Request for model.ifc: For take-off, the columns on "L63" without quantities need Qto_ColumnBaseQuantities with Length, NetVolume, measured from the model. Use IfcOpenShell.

First a look at what the model holds.

```python
import ifcopenshell
import ifcopenshell.util.element
import ifcopenshell.util.unit

model = ifcopenshell.open("model.ifc")
print(model.schema)
for unit_type in ("LENGTHUNIT", "AREAUNIT", "VOLUMEUNIT"):
    print(unit_type, ifcopenshell.util.unit.calculate_unit_scale(model, unit_type))
storey = next(s for s in model.by_type("IfcBuildingStorey") if s.Name == "L63")
columns = [e for e in ifcopenshell.util.element.get_decomposition(storey) if e.is_a("IfcColumn")]
for e in sorted(columns, key=lambda e: e.id()):
    print(e.id(), e.is_a(), e.Name, list(ifcopenshell.util.element.get_psets(e, qtos_only=True)), sep=" | ")
```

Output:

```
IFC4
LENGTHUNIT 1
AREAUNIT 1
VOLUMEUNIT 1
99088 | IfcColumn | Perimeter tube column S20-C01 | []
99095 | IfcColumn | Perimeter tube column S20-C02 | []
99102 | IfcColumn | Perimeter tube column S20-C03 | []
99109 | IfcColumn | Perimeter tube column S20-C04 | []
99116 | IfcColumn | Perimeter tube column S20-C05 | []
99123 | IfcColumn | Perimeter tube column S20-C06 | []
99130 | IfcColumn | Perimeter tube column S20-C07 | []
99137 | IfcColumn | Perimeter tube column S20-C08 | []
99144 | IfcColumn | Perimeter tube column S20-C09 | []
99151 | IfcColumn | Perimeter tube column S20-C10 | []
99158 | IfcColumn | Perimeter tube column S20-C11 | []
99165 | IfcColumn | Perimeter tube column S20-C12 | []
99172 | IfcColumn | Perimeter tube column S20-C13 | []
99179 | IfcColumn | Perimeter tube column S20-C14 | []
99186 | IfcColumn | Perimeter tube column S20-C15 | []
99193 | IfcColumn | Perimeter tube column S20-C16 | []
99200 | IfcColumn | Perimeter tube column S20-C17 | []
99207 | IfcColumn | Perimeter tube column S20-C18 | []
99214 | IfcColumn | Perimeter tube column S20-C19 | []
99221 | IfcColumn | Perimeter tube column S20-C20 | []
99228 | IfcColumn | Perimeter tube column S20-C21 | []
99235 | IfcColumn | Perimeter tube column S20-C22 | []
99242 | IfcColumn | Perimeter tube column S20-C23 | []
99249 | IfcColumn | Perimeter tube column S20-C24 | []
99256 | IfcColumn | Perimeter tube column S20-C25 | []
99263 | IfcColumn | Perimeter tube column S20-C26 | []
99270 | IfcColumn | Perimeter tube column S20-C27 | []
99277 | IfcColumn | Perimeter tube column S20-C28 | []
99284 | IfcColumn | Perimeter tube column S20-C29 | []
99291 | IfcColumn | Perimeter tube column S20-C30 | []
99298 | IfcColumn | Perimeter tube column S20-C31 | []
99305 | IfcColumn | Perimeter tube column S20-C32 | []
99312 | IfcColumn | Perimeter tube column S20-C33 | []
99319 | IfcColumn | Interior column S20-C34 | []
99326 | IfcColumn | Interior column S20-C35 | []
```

```python
import ifcopenshell
import ifcopenshell.api.pset
import ifcopenshell.geom
import ifcopenshell.util.element
import ifcopenshell.util.shape
import ifcopenshell.util.unit

model = ifcopenshell.open("model.ifc")
unit_scale = ifcopenshell.util.unit.calculate_unit_scale(model)
volume_scale = ifcopenshell.util.unit.calculate_unit_scale(model, "VOLUMEUNIT")
settings = ifcopenshell.geom.settings()

storey = next(s for s in model.by_type("IfcBuildingStorey") if s.Name == "L63")
columns = [e for e in ifcopenshell.util.element.get_decomposition(storey) if e.is_a("IfcColumn")]

for e in sorted(columns, key=lambda e: e.id()):
    if ifcopenshell.util.element.get_psets(e, qtos_only=True, should_inherit=False):
        continue
    # Geometry comes back in metres, in the element's own axes.
    shape = ifcopenshell.geom.create_shape(settings, e)
    values = {
        "Length": ifcopenshell.util.shape.get_z(shape.geometry) / unit_scale,
        "NetVolume": ifcopenshell.util.shape.get_volume(shape.geometry) / volume_scale,
    }
    qto = ifcopenshell.api.pset.add_qto(model, product=e, name="Qto_ColumnBaseQuantities")
    ifcopenshell.api.pset.edit_qto(model, qto=qto, properties=values)
    print(e.id(), {k: round(v, 3) for k, v in values.items()})

model.write("model_edited.ifc")
```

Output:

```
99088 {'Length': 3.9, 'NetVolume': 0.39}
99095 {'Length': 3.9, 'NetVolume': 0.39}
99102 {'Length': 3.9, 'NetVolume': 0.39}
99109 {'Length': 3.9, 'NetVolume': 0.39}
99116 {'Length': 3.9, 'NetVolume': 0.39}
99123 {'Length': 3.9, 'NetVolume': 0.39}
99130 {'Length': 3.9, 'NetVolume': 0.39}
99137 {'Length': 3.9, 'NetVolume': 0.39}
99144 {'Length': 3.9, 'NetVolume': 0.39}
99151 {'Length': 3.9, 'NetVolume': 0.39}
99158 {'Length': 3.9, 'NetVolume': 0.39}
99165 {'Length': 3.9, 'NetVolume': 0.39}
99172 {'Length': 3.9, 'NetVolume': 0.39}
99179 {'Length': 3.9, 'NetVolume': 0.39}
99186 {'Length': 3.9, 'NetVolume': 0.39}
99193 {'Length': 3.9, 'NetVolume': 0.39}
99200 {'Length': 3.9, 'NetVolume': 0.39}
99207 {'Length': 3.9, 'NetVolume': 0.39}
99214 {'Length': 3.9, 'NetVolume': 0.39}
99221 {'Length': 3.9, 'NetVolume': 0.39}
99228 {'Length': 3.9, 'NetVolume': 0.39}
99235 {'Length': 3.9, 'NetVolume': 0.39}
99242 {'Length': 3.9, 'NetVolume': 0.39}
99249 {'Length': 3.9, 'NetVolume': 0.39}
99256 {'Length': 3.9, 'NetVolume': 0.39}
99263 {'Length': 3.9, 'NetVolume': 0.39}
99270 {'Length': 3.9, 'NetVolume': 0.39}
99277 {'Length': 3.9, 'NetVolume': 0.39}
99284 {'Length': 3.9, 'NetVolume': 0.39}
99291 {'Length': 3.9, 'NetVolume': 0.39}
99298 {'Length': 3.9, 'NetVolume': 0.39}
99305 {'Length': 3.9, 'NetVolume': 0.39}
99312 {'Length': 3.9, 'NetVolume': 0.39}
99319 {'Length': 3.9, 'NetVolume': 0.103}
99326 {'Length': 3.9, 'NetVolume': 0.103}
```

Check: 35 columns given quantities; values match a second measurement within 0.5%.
